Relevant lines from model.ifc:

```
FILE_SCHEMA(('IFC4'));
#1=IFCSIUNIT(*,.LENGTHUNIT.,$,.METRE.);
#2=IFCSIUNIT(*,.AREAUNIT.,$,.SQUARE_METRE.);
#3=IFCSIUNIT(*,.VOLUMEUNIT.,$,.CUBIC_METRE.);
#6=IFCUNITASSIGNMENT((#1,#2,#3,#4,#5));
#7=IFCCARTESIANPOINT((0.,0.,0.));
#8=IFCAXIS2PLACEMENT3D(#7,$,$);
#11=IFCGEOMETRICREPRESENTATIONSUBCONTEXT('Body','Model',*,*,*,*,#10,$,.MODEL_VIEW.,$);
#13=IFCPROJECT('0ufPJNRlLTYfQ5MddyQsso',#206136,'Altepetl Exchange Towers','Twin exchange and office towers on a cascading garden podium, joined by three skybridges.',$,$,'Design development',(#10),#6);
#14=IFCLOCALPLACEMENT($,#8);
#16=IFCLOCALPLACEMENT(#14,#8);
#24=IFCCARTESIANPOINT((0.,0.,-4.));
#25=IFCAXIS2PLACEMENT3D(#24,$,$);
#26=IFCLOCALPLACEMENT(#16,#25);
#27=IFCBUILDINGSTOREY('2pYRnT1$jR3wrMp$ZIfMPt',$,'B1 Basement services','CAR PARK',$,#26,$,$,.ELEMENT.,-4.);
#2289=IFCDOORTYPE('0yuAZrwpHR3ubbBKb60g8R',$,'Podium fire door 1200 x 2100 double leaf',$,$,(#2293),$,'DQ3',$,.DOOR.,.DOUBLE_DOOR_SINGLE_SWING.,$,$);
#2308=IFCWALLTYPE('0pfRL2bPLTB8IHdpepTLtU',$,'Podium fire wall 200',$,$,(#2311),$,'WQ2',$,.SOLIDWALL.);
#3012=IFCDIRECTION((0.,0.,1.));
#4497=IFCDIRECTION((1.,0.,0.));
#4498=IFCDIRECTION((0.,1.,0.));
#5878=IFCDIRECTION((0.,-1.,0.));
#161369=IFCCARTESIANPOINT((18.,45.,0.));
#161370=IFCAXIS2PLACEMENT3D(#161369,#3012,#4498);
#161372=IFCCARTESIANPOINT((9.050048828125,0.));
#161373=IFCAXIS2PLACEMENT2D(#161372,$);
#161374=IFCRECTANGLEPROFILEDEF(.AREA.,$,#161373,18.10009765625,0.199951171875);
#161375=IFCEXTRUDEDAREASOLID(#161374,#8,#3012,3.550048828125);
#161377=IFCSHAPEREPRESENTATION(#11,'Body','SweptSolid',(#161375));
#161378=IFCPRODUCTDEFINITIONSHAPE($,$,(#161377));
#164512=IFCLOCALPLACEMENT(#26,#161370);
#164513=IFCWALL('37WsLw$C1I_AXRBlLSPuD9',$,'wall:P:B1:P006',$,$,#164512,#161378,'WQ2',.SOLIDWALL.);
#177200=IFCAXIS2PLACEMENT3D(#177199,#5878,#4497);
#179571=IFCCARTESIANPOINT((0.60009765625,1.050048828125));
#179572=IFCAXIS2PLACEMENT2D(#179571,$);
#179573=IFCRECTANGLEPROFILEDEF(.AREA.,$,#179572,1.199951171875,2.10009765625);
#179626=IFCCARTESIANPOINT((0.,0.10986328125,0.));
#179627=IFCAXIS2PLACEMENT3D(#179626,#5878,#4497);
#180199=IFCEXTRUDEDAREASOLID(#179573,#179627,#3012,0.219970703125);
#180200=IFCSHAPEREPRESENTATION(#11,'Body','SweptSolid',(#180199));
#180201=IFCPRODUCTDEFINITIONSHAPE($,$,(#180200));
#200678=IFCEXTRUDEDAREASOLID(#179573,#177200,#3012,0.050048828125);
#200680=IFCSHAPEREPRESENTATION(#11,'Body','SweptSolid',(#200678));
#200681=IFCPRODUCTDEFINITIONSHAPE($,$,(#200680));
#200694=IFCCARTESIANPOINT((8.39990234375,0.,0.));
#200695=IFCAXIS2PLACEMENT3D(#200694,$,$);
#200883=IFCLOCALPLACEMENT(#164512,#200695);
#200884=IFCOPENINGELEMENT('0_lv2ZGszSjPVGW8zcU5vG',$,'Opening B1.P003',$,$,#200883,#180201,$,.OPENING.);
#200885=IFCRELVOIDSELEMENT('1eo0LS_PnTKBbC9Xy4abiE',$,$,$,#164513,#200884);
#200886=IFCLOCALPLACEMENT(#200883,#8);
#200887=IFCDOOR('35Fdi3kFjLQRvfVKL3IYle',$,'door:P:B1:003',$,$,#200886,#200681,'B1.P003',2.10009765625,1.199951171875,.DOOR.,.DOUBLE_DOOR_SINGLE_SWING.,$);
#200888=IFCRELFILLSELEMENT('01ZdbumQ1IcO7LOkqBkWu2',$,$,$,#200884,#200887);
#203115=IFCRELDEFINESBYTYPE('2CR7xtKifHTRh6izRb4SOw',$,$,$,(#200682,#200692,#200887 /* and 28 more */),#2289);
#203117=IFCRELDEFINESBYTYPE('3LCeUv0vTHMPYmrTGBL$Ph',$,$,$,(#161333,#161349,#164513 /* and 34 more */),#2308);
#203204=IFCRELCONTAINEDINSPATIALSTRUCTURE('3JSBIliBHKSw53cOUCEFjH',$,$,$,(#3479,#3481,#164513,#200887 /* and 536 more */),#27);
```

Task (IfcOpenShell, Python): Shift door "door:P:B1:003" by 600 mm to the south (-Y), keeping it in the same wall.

```python
import ifcopenshell
import ifcopenshell.api.geometry
import ifcopenshell.util.placement
import ifcopenshell.util.unit

model = ifcopenshell.open("model.ifc")
unit_scale = ifcopenshell.util.unit.calculate_unit_scale(model)

door = model.by_guid("35Fdi3kFjLQRvfVKL3IYle")
opening = door.FillsVoids[0].RelatingOpeningElement
wall = opening.VoidsElements[0].RelatingBuildingElement

wall_matrix = ifcopenshell.util.placement.get_local_placement(wall.ObjectPlacement)
shift = wall_matrix[:3, 0] * -0.6 / unit_scale
before = ifcopenshell.util.placement.get_local_placement(door.ObjectPlacement)[:3, 3].copy()

# The door is placed relative to its opening, so it follows when the opening moves.
matrix = ifcopenshell.util.placement.get_local_placement(opening.ObjectPlacement)
matrix[:3, 3] += shift
ifcopenshell.api.geometry.edit_object_placement(
    model, product=opening, matrix=matrix, is_si=False, should_transform_children=True
)

after = ifcopenshell.util.placement.get_local_placement(door.ObjectPlacement)[:3, 3]
print("door moved by", (after - before).round(3) + 0.0)

model.write("model_v2.ifc")
```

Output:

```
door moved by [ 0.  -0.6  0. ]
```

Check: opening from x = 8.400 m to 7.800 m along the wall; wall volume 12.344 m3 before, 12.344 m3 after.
